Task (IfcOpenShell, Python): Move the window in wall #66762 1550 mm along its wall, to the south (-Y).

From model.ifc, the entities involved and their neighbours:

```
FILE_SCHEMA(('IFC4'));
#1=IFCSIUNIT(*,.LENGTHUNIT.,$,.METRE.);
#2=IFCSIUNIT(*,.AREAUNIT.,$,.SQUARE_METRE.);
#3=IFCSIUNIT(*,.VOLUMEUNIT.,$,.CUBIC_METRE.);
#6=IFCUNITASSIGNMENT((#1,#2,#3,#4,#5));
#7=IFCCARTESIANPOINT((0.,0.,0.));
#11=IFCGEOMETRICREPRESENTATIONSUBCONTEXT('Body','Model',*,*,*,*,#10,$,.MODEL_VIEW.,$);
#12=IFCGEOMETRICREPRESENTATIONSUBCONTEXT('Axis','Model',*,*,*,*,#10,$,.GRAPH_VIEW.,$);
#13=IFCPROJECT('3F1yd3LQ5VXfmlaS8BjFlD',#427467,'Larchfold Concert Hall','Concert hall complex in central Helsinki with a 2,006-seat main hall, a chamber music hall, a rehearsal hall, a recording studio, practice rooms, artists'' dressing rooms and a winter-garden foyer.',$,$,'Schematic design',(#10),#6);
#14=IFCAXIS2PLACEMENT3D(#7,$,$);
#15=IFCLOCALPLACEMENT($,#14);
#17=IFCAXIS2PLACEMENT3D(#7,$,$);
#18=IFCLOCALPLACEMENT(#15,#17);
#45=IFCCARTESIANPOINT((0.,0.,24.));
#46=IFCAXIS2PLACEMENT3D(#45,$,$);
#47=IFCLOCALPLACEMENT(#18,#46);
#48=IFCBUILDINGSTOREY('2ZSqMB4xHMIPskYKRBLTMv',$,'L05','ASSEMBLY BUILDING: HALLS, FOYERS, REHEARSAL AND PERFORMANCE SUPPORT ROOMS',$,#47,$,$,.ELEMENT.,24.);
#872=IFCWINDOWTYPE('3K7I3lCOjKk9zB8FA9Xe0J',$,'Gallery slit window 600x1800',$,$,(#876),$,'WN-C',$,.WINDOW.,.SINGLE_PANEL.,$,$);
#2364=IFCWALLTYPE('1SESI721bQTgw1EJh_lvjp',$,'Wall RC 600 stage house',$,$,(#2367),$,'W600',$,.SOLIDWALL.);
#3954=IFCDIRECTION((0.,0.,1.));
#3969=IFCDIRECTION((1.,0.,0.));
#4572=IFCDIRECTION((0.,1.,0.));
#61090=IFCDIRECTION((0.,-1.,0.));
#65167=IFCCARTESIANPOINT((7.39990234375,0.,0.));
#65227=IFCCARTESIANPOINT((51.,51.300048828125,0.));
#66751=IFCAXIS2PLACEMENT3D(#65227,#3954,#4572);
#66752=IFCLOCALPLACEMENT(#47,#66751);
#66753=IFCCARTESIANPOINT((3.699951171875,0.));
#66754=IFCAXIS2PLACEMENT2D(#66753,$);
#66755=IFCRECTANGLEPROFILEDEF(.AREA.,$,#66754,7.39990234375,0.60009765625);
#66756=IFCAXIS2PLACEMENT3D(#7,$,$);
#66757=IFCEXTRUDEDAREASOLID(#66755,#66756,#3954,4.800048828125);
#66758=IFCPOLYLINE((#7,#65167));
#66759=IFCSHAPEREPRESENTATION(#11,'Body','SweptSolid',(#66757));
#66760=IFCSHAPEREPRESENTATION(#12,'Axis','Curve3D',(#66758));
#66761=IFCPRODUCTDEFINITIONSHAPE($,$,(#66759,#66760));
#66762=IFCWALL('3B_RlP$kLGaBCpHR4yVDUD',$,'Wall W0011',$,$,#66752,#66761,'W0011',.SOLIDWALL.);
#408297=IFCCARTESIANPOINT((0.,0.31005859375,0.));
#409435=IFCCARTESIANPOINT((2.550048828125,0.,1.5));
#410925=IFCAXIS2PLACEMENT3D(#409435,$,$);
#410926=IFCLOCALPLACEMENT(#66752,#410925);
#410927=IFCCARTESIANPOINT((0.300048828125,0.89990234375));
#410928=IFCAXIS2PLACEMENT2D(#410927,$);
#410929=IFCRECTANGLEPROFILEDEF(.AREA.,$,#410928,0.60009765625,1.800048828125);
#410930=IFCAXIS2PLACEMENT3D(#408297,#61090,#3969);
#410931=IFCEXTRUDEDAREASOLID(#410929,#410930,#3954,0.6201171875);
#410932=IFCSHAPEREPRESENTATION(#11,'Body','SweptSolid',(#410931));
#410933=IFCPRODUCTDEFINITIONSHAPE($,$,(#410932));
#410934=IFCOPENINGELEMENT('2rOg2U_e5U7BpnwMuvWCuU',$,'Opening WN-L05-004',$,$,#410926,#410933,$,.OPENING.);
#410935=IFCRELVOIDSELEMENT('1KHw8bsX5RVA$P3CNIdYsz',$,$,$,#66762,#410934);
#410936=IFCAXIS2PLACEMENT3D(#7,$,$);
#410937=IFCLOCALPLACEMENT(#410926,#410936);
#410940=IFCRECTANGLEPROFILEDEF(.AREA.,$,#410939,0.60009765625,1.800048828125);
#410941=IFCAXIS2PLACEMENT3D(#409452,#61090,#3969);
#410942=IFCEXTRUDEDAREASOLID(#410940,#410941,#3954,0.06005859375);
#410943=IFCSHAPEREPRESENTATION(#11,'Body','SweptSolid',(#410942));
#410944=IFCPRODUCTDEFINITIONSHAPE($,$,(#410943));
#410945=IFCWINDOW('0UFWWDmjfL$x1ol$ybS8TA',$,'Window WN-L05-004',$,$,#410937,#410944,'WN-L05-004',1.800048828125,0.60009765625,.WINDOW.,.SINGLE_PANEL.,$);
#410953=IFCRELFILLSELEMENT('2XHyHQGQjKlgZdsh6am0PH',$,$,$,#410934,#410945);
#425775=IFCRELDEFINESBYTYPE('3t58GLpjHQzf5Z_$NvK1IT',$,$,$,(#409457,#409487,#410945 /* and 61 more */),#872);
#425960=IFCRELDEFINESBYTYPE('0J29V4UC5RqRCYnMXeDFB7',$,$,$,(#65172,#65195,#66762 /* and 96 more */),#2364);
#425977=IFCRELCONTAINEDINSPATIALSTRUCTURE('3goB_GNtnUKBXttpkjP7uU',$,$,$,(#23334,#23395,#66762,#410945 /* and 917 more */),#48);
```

```python
import ifcopenshell
import ifcopenshell.api.geometry
import ifcopenshell.util.placement
import ifcopenshell.util.unit

model = ifcopenshell.open("model.ifc")
unit_scale = ifcopenshell.util.unit.calculate_unit_scale(model)

window = model.by_guid("0UFWWDmjfL$x1ol$ybS8TA")
opening = window.FillsVoids[0].RelatingOpeningElement
wall = opening.VoidsElements[0].RelatingBuildingElement

wall_matrix = ifcopenshell.util.placement.get_local_placement(wall.ObjectPlacement)
shift = wall_matrix[:3, 0] * -1.55 / unit_scale
before = ifcopenshell.util.placement.get_local_placement(window.ObjectPlacement)[:3, 3].copy()

# The window is placed relative to its opening, so it follows when the opening moves.
matrix = ifcopenshell.util.placement.get_local_placement(opening.ObjectPlacement)
matrix[:3, 3] += shift
ifcopenshell.api.geometry.edit_object_placement(
    model, product=opening, matrix=matrix, is_si=False, should_transform_children=True
)

after = ifcopenshell.util.placement.get_local_placement(window.ObjectPlacement)[:3, 3]
print("window moved by", (after - before).round(3) + 0.0)

model.write("model_v2.ifc")
```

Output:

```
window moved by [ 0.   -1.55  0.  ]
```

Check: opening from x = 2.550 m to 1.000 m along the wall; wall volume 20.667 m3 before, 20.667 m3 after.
